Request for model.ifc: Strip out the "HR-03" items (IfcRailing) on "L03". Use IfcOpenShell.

First a look at what the model holds.

```python
import ifcopenshell
import ifcopenshell.util.element

model = ifcopenshell.open("model.ifc")
print(model.schema)
storey = next(s for s in model.by_type("IfcBuildingStorey") if s.Name == "L03")
railings = [e for e in ifcopenshell.util.element.get_decomposition(storey) if e.is_a("IfcRailing")]
seen = {}
for e in railings:
    element_type = ifcopenshell.util.element.get_type(e)
    name = element_type.Name if element_type not in (None, e) else None
    seen[name] = seen.get(name, 0) + 1
for name, count in sorted(seen.items(), key=str):
    print(count, "x", name)
```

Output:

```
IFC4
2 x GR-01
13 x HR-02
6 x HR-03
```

```python
import ifcopenshell
import ifcopenshell.api.root
import ifcopenshell.util.element

model = ifcopenshell.open("model.ifc")

storey = next(s for s in model.by_type("IfcBuildingStorey") if s.Name == "L03")
railings = [e for e in ifcopenshell.util.element.get_decomposition(storey) if e.is_a("IfcRailing")]
targets = [e for e in railings if (t := ifcopenshell.util.element.get_type(e)) not in (None, e) and t.Name == "HR-03"]

for e in targets:
    ifcopenshell.api.root.remove_product(model, product=e)
print(len(targets), "removed")

model.write("model_v2.ifc")
```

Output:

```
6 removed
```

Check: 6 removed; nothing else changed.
